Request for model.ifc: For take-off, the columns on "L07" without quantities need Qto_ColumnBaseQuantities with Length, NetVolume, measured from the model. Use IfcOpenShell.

First a look at what the model holds.

```python
import ifcopenshell
import ifcopenshell.util.element
import ifcopenshell.util.unit

model = ifcopenshell.open("model.ifc")
print(model.schema)
for unit_type in ("LENGTHUNIT", "AREAUNIT", "VOLUMEUNIT"):
    print(unit_type, ifcopenshell.util.unit.calculate_unit_scale(model, unit_type))
storey = next(s for s in model.by_type("IfcBuildingStorey") if s.Name == "L07")
columns = [e for e in ifcopenshell.util.element.get_decomposition(storey) if e.is_a("IfcColumn")]
for e in sorted(columns, key=lambda e: e.id()):
    print(e.id(), e.is_a(), e.Name, list(ifcopenshell.util.element.get_psets(e, qtos_only=True)), sep=" | ")
```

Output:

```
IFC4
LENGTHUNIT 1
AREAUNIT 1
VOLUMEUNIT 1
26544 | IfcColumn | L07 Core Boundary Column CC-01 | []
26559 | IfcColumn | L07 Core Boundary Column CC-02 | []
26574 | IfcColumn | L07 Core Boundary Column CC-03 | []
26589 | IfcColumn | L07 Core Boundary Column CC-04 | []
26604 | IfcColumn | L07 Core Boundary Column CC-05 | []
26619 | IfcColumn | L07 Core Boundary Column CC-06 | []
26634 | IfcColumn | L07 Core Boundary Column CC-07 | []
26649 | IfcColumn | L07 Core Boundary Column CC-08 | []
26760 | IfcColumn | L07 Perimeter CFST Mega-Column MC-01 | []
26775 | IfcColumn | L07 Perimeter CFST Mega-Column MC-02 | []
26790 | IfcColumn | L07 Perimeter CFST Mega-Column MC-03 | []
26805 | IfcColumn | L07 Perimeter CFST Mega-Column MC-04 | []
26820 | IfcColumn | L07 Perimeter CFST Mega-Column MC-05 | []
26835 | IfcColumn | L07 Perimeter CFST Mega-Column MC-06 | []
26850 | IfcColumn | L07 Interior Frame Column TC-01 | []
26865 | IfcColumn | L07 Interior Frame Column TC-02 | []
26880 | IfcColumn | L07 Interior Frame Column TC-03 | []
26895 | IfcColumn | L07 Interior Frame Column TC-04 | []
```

```python
import ifcopenshell
import ifcopenshell.api.pset
import ifcopenshell.geom
import ifcopenshell.util.element
import ifcopenshell.util.shape
import ifcopenshell.util.unit

model = ifcopenshell.open("model.ifc")
unit_scale = ifcopenshell.util.unit.calculate_unit_scale(model)
volume_scale = ifcopenshell.util.unit.calculate_unit_scale(model, "VOLUMEUNIT")
settings = ifcopenshell.geom.settings()

storey = next(s for s in model.by_type("IfcBuildingStorey") if s.Name == "L07")
columns = [e for e in ifcopenshell.util.element.get_decomposition(storey) if e.is_a("IfcColumn")]

for e in sorted(columns, key=lambda e: e.id()):
    if ifcopenshell.util.element.get_psets(e, qtos_only=True, should_inherit=False):
        continue
    # Geometry comes back in metres, in the element's own axes.
    shape = ifcopenshell.geom.create_shape(settings, e)
    values = {
        "Length": ifcopenshell.util.shape.get_z(shape.geometry) / unit_scale,
        "NetVolume": ifcopenshell.util.shape.get_volume(shape.geometry) / volume_scale,
    }
    qto = ifcopenshell.api.pset.add_qto(model, product=e, name="Qto_ColumnBaseQuantities")
    ifcopenshell.api.pset.edit_qto(model, qto=qto, properties=values)
    print(e.id(), {k: round(v, 3) for k, v in values.items()})

model.write("model_rev.ifc")
```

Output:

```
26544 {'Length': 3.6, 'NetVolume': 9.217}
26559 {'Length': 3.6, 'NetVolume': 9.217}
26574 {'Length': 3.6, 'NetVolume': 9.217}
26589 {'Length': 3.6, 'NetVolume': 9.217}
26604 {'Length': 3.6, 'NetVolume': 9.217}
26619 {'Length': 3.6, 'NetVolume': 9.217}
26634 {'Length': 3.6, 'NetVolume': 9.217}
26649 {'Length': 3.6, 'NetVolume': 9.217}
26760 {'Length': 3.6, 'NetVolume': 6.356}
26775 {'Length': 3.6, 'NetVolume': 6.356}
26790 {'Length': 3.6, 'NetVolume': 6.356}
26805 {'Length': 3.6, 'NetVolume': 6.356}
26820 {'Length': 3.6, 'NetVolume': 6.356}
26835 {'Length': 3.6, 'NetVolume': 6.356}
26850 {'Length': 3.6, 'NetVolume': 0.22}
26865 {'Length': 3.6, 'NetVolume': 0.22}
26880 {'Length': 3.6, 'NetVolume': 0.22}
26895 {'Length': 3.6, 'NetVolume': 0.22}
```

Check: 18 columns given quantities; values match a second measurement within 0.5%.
